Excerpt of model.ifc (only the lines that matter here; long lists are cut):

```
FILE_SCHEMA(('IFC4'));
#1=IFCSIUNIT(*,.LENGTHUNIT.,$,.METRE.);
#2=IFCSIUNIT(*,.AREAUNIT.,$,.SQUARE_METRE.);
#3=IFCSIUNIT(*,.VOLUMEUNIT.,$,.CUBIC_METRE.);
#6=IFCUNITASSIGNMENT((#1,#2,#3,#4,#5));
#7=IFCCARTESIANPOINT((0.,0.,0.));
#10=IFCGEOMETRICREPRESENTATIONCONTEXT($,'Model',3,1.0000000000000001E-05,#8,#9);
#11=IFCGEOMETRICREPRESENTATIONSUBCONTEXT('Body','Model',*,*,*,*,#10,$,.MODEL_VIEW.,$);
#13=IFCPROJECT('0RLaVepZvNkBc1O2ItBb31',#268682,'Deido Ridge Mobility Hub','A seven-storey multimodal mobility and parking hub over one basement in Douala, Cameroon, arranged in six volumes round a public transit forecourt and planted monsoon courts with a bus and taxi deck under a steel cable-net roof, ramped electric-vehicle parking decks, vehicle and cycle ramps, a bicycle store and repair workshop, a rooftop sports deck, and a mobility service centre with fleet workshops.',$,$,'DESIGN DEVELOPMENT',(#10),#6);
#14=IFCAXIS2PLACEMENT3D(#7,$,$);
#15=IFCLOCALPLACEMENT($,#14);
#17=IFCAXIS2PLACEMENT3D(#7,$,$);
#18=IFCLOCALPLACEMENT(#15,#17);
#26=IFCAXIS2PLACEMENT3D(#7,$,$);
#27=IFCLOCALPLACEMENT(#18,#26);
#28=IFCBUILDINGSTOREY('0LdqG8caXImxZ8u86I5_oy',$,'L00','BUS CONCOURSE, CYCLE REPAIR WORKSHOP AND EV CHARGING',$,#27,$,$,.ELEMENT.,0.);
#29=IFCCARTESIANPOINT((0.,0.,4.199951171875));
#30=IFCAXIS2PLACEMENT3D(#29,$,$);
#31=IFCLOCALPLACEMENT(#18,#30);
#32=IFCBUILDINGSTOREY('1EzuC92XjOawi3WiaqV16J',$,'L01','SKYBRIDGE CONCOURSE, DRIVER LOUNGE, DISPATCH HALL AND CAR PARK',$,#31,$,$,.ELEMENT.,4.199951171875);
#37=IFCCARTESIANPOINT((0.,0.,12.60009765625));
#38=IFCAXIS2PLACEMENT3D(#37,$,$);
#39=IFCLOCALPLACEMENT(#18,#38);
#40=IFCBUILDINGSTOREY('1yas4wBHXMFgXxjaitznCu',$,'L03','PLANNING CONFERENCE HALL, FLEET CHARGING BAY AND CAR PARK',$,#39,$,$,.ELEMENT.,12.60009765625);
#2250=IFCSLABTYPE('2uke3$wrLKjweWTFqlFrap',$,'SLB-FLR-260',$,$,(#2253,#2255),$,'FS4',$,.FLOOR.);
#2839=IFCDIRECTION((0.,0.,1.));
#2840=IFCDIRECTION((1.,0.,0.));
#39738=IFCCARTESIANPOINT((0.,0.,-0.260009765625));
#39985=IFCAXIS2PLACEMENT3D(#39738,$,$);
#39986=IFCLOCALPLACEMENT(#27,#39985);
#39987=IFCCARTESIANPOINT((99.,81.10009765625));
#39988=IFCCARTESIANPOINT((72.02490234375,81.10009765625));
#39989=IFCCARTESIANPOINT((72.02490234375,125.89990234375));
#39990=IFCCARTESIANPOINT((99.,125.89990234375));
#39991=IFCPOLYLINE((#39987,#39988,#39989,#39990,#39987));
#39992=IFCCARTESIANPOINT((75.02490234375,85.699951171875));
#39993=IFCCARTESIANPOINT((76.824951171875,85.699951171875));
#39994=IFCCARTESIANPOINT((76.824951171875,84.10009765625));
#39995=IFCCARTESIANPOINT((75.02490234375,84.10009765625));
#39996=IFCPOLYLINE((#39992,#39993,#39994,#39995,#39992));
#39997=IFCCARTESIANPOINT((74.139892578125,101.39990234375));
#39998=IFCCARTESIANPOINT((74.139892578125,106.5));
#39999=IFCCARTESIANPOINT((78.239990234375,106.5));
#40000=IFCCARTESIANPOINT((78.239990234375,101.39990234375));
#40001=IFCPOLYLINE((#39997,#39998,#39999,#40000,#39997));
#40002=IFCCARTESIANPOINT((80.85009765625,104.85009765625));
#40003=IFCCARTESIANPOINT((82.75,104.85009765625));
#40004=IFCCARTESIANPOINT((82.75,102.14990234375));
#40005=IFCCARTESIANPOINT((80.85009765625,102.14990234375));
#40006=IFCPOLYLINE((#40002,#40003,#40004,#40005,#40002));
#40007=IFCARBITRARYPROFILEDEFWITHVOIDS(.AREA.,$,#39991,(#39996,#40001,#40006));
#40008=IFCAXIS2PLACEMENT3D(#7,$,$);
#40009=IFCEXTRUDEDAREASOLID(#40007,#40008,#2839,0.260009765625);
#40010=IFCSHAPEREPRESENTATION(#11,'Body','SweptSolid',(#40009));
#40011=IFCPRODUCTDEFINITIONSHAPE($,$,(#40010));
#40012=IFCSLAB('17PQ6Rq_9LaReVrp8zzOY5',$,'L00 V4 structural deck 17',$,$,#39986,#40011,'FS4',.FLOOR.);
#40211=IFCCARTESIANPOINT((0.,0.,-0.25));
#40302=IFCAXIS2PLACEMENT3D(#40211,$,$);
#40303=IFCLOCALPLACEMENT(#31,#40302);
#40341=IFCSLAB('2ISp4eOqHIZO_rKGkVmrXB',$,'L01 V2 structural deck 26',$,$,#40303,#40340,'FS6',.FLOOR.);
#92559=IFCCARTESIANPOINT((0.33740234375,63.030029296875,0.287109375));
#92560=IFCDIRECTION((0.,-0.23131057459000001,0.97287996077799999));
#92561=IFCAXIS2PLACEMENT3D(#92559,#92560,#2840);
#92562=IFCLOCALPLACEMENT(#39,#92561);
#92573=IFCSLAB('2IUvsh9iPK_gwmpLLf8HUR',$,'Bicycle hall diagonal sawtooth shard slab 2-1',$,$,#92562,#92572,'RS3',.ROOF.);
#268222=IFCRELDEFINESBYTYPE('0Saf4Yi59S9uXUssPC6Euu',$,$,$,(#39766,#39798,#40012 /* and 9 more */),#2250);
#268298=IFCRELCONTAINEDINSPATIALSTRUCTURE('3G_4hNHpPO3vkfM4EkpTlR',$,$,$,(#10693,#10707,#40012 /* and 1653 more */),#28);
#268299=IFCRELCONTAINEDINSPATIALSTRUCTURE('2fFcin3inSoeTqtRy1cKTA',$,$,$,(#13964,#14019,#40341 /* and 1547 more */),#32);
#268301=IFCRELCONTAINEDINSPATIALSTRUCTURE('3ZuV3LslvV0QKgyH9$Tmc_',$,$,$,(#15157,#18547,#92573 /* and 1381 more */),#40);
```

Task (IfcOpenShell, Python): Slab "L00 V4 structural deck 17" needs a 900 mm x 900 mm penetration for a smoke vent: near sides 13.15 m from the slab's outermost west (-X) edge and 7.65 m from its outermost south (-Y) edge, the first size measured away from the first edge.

```python
import numpy as np
import ifcopenshell
import ifcopenshell.api.feature
import ifcopenshell.api.geometry
import ifcopenshell.api.root
import ifcopenshell.geom
import ifcopenshell.util.placement
import ifcopenshell.util.representation
import ifcopenshell.util.shape
import ifcopenshell.util.unit

model = ifcopenshell.open("model.ifc")
unit_scale = ifcopenshell.util.unit.calculate_unit_scale(model)
settings = ifcopenshell.geom.settings()


def volume(element):
    """Net volume in cubic metres, openings subtracted."""
    shape = ifcopenshell.geom.create_shape(settings, element)
    return ifcopenshell.util.shape.get_volume(shape.geometry)


slab = model.by_id(40012)
before = volume(slab)

# Extent in the slab's own axes, in metres. The edges named are its -X and -Y sides.
slab_shape = ifcopenshell.geom.create_shape(settings, slab)
vertices = ifcopenshell.util.shape.get_vertices(slab_shape.geometry)
x_min, y_min, bottom = vertices.min(axis=0)
top = vertices[:, 2].max()

opening = ifcopenshell.api.root.create_entity(model, ifc_class="IfcOpeningElement", name="Smoke vent opening", predefined_type="OPENING")
context = ifcopenshell.util.representation.get_context(model, "Model", "Body", "MODEL_VIEW")
width, depth = 0.9, 0.9
outline = [(0.0, 0.0), (width, 0.0), (width, depth), (0.0, depth), (0.0, 0.0)]
# Overshoot both faces by 50 mm so the cut is clean.
shape = ifcopenshell.api.geometry.add_slab_representation(
    model, context=context, depth=top - bottom + 0.1, polyline=outline
)
ifcopenshell.api.geometry.assign_representation(model, product=opening, representation=shape)

matrix = ifcopenshell.util.placement.get_local_placement(slab.ObjectPlacement)
matrix[:, 3] = matrix @ np.append(np.array([x_min + 13.15, y_min + 7.65, bottom - 0.05]) / unit_scale, 1.0)
ifcopenshell.api.geometry.edit_object_placement(model, product=opening, matrix=matrix, is_si=False)
ifcopenshell.api.feature.add_feature(model, feature=opening, element=slab)

after = volume(slab)

print(f"slab volume {before:.3f} -> {after:.3f} m3")

model.write("model_v2.ifc")
```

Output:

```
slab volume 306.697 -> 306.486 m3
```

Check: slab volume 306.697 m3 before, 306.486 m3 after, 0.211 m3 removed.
